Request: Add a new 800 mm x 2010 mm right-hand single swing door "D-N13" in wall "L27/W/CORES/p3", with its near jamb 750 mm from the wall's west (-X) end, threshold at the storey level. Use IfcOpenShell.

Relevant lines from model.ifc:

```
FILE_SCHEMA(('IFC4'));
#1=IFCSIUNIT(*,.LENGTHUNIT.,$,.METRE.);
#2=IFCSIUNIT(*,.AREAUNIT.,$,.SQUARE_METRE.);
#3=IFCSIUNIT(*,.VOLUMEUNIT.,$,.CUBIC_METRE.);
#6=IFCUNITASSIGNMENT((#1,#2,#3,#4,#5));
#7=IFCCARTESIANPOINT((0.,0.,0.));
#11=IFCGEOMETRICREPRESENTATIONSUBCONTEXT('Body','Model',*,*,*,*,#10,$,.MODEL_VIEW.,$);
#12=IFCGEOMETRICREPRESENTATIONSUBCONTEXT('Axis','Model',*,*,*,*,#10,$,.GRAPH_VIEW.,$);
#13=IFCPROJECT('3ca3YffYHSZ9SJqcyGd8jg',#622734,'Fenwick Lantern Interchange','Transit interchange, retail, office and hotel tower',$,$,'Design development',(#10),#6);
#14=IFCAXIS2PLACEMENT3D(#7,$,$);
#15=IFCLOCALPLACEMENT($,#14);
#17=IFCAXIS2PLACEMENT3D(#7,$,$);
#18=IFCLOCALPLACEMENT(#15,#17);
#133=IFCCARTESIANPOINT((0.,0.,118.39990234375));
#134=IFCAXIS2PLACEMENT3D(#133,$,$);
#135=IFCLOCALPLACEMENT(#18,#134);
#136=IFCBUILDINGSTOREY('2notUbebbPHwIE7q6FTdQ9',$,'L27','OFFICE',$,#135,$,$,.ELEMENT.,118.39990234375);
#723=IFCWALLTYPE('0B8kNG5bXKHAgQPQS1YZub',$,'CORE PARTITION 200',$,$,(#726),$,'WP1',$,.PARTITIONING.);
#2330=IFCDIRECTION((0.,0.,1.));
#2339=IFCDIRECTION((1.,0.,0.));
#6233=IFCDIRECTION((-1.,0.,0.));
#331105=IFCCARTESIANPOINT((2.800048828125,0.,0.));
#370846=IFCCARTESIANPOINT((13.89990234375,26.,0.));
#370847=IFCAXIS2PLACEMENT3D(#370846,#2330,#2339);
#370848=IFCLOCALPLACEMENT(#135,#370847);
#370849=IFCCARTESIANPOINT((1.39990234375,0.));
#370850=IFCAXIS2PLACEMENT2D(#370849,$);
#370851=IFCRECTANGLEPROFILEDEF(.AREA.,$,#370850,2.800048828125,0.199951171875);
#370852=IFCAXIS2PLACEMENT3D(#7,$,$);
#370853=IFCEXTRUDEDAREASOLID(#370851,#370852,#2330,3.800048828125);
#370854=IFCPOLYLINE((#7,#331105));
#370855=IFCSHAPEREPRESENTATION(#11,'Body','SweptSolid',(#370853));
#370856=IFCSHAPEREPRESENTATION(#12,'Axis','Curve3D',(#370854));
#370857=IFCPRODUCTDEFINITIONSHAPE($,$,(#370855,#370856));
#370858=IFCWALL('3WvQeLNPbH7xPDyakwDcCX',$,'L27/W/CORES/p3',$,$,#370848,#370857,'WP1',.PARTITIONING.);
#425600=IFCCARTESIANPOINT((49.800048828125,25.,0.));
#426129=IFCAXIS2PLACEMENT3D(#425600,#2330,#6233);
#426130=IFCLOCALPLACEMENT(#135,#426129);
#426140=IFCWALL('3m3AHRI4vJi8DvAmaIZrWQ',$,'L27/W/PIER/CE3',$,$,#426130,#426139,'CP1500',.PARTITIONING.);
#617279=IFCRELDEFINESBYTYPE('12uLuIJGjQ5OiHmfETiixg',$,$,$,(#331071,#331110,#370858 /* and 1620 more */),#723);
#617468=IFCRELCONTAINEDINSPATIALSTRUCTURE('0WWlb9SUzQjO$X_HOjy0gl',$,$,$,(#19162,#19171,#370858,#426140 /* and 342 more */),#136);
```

```python
import numpy as np
import ifcopenshell
import ifcopenshell.api.feature
import ifcopenshell.api.geometry
import ifcopenshell.api.root
import ifcopenshell.api.spatial
import ifcopenshell.geom
import ifcopenshell.util.element
import ifcopenshell.util.placement
import ifcopenshell.util.representation
import ifcopenshell.util.shape
import ifcopenshell.util.unit

model = ifcopenshell.open("model.ifc")
unit_scale = ifcopenshell.util.unit.calculate_unit_scale(model)
settings = ifcopenshell.geom.settings()


def volume(element):
    """Net volume in cubic metres, openings subtracted."""
    shape = ifcopenshell.geom.create_shape(settings, element)
    return ifcopenshell.util.shape.get_volume(shape.geometry)


wall = model.by_guid("3WvQeLNPbH7xPDyakwDcCX")
storey = ifcopenshell.util.element.get_container(wall, ifc_class="IfcBuildingStorey")
context = ifcopenshell.util.representation.get_context(model, "Model", "Body", "MODEL_VIEW")
before = volume(wall)

width, height, from_end, sill = 0.8, 2.01, 0.75, 0.0  # metres

# The wall runs along its own X axis, and the end named is its -X end.
wall_shape = ifcopenshell.geom.create_shape(settings, wall)
x, y, z = ifcopenshell.util.shape.get_vertices(wall_shape.geometry).T
start = x.min() + from_end
face, thickness = float(y.min()), float(y.max() - y.min())
wall_matrix = ifcopenshell.util.placement.get_local_placement(wall.ObjectPlacement)
level = ifcopenshell.util.placement.get_local_placement(storey.ObjectPlacement)[2, 3]


def in_wall(x, y):
    """Placement at x, y metres in the wall's axes, at sill height."""
    matrix = wall_matrix.copy()
    matrix[:, 3] = wall_matrix @ np.array([x / unit_scale, y / unit_scale, 0.0, 1.0])
    matrix[2, 3] = level + sill / unit_scale
    return matrix


# Opening: a box that overshoots both wall faces by 50 mm.
opening = ifcopenshell.api.root.create_entity(model, ifc_class="IfcOpeningElement", predefined_type="OPENING")
box = ifcopenshell.api.geometry.add_wall_representation(
    model, context=context, length=width, height=height, thickness=thickness + 0.1
)
ifcopenshell.api.geometry.assign_representation(model, product=opening, representation=box)
ifcopenshell.api.geometry.edit_object_placement(model, product=opening, matrix=in_wall(start, face - 0.05), is_si=False)
ifcopenshell.api.feature.add_feature(model, feature=opening, element=wall)

door = ifcopenshell.api.root.create_entity(model, ifc_class="IfcDoor", name="D-N13", predefined_type="DOOR")
door.OverallWidth, door.OverallHeight = width / unit_scale, height / unit_scale
door.OperationType = "SINGLE_SWING_RIGHT"
body = ifcopenshell.api.geometry.add_door_representation(
    model,
    context=context,
    overall_width=door.OverallWidth,
    overall_height=door.OverallHeight,
    operation_type="SINGLE_SWING_RIGHT",
    lining_properties={"LiningDepth": thickness / unit_scale, "ThresholdDepth": thickness / unit_scale},
)
ifcopenshell.api.geometry.assign_representation(model, product=door, representation=body)
ifcopenshell.api.spatial.assign_container(model, products=[door], relating_structure=storey)
ifcopenshell.api.feature.add_filling(model, opening=opening, element=door)

# The lining spans the wall, so the door starts at the wall face.
ifcopenshell.api.geometry.edit_object_placement(model, product=door, matrix=in_wall(start, face), is_si=False)

after = volume(wall)

print(f"wall volume {before:.3f} -> {after:.3f} m3")

model.write("model_updated.ifc")
```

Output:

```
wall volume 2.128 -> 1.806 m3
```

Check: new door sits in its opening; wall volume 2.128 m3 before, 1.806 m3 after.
